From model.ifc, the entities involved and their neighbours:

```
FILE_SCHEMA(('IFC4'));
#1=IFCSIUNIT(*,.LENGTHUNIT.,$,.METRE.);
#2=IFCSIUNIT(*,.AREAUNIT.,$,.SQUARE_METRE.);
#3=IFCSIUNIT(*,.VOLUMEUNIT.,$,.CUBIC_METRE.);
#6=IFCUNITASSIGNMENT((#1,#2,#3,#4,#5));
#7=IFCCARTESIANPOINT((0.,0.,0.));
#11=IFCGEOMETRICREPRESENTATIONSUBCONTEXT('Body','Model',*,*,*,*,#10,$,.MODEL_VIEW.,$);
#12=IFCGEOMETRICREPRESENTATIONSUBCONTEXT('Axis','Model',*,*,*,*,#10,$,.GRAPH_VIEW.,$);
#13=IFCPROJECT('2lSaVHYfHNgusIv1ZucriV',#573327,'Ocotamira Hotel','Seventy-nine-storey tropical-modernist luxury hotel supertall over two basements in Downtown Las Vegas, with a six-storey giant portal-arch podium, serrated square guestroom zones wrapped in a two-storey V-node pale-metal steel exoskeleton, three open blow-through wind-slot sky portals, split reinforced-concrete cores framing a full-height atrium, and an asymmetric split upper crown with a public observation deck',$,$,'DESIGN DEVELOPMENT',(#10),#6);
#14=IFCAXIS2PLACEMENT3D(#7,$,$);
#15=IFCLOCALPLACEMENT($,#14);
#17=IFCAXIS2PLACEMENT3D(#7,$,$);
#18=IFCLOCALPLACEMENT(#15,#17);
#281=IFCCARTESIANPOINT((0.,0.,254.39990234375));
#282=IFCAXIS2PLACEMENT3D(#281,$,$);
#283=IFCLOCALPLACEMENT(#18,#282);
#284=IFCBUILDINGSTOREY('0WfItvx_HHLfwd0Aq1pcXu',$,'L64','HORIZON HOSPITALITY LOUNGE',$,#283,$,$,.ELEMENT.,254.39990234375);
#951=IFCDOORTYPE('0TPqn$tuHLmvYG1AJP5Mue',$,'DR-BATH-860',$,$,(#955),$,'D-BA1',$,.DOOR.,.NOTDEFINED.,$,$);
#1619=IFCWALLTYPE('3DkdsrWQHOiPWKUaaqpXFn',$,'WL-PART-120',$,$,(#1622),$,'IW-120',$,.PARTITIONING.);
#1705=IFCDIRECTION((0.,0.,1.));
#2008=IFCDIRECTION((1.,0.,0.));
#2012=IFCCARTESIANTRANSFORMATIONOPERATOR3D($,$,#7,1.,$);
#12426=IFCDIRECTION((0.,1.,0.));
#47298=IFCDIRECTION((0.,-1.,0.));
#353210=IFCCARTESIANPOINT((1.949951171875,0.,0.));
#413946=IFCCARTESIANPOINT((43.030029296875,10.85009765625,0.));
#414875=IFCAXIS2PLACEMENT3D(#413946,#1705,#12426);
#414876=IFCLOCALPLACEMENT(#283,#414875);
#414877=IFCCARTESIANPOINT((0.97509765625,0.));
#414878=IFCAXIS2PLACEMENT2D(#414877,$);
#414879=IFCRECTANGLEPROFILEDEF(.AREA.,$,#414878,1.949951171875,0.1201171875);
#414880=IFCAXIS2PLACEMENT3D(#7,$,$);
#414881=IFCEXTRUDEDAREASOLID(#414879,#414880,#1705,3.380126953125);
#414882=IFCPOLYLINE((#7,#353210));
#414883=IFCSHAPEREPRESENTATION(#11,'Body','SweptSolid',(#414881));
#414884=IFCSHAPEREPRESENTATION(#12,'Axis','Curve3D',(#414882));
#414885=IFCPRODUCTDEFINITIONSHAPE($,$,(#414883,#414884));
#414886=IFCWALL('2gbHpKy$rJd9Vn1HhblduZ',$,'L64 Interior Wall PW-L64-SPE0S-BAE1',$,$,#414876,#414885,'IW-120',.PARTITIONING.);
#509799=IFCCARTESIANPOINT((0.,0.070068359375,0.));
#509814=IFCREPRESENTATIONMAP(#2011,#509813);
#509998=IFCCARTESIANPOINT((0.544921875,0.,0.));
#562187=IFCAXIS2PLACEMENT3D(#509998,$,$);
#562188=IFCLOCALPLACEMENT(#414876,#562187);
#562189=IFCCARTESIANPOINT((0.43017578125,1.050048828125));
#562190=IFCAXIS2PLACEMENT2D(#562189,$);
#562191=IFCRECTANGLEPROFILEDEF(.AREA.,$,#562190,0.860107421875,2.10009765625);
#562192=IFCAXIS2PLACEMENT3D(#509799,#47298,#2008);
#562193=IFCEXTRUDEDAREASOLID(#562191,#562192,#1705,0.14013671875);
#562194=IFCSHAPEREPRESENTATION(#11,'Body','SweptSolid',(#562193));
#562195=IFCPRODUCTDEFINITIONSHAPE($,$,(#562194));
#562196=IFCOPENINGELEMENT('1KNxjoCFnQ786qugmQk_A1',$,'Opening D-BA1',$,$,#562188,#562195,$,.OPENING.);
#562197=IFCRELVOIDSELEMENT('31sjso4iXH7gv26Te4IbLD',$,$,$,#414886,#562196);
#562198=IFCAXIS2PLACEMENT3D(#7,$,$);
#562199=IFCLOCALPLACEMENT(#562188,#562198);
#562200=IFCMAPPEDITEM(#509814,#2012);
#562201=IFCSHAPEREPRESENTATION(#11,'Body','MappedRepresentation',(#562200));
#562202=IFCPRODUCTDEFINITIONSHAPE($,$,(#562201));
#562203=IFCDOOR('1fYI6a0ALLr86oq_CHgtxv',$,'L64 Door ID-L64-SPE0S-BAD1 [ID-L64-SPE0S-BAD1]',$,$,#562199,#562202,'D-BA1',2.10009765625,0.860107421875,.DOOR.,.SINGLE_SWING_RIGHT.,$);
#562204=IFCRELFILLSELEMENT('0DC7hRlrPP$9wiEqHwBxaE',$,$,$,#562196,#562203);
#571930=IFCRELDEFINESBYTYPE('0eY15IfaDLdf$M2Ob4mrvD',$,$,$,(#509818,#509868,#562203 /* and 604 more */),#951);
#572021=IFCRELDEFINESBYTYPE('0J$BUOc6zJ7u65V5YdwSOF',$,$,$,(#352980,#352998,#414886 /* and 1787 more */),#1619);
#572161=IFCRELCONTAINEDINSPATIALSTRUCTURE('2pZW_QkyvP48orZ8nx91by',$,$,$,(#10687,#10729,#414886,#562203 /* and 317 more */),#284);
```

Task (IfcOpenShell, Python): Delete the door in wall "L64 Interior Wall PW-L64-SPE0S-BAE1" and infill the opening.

```python
import ifcopenshell
import ifcopenshell.api.feature
import ifcopenshell.api.root
import ifcopenshell.geom
import ifcopenshell.util.shape

model = ifcopenshell.open("model.ifc")
settings = ifcopenshell.geom.settings()


def volume(element):
    """Net volume in cubic metres, openings subtracted."""
    shape = ifcopenshell.geom.create_shape(settings, element)
    return ifcopenshell.util.shape.get_volume(shape.geometry)


door = model.by_guid("1fYI6a0ALLr86oq_CHgtxv")
opening = door.FillsVoids[0].RelatingOpeningElement
wall = opening.VoidsElements[0].RelatingBuildingElement
before = volume(wall)

ifcopenshell.api.root.remove_product(model, product=door)
ifcopenshell.api.feature.remove_feature(model, feature=opening)

after = volume(wall)

print(f"wall volume {before:.3f} -> {after:.3f} m3")

model.write("model_updated.ifc")
```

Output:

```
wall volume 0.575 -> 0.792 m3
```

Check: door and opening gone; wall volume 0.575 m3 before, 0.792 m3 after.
